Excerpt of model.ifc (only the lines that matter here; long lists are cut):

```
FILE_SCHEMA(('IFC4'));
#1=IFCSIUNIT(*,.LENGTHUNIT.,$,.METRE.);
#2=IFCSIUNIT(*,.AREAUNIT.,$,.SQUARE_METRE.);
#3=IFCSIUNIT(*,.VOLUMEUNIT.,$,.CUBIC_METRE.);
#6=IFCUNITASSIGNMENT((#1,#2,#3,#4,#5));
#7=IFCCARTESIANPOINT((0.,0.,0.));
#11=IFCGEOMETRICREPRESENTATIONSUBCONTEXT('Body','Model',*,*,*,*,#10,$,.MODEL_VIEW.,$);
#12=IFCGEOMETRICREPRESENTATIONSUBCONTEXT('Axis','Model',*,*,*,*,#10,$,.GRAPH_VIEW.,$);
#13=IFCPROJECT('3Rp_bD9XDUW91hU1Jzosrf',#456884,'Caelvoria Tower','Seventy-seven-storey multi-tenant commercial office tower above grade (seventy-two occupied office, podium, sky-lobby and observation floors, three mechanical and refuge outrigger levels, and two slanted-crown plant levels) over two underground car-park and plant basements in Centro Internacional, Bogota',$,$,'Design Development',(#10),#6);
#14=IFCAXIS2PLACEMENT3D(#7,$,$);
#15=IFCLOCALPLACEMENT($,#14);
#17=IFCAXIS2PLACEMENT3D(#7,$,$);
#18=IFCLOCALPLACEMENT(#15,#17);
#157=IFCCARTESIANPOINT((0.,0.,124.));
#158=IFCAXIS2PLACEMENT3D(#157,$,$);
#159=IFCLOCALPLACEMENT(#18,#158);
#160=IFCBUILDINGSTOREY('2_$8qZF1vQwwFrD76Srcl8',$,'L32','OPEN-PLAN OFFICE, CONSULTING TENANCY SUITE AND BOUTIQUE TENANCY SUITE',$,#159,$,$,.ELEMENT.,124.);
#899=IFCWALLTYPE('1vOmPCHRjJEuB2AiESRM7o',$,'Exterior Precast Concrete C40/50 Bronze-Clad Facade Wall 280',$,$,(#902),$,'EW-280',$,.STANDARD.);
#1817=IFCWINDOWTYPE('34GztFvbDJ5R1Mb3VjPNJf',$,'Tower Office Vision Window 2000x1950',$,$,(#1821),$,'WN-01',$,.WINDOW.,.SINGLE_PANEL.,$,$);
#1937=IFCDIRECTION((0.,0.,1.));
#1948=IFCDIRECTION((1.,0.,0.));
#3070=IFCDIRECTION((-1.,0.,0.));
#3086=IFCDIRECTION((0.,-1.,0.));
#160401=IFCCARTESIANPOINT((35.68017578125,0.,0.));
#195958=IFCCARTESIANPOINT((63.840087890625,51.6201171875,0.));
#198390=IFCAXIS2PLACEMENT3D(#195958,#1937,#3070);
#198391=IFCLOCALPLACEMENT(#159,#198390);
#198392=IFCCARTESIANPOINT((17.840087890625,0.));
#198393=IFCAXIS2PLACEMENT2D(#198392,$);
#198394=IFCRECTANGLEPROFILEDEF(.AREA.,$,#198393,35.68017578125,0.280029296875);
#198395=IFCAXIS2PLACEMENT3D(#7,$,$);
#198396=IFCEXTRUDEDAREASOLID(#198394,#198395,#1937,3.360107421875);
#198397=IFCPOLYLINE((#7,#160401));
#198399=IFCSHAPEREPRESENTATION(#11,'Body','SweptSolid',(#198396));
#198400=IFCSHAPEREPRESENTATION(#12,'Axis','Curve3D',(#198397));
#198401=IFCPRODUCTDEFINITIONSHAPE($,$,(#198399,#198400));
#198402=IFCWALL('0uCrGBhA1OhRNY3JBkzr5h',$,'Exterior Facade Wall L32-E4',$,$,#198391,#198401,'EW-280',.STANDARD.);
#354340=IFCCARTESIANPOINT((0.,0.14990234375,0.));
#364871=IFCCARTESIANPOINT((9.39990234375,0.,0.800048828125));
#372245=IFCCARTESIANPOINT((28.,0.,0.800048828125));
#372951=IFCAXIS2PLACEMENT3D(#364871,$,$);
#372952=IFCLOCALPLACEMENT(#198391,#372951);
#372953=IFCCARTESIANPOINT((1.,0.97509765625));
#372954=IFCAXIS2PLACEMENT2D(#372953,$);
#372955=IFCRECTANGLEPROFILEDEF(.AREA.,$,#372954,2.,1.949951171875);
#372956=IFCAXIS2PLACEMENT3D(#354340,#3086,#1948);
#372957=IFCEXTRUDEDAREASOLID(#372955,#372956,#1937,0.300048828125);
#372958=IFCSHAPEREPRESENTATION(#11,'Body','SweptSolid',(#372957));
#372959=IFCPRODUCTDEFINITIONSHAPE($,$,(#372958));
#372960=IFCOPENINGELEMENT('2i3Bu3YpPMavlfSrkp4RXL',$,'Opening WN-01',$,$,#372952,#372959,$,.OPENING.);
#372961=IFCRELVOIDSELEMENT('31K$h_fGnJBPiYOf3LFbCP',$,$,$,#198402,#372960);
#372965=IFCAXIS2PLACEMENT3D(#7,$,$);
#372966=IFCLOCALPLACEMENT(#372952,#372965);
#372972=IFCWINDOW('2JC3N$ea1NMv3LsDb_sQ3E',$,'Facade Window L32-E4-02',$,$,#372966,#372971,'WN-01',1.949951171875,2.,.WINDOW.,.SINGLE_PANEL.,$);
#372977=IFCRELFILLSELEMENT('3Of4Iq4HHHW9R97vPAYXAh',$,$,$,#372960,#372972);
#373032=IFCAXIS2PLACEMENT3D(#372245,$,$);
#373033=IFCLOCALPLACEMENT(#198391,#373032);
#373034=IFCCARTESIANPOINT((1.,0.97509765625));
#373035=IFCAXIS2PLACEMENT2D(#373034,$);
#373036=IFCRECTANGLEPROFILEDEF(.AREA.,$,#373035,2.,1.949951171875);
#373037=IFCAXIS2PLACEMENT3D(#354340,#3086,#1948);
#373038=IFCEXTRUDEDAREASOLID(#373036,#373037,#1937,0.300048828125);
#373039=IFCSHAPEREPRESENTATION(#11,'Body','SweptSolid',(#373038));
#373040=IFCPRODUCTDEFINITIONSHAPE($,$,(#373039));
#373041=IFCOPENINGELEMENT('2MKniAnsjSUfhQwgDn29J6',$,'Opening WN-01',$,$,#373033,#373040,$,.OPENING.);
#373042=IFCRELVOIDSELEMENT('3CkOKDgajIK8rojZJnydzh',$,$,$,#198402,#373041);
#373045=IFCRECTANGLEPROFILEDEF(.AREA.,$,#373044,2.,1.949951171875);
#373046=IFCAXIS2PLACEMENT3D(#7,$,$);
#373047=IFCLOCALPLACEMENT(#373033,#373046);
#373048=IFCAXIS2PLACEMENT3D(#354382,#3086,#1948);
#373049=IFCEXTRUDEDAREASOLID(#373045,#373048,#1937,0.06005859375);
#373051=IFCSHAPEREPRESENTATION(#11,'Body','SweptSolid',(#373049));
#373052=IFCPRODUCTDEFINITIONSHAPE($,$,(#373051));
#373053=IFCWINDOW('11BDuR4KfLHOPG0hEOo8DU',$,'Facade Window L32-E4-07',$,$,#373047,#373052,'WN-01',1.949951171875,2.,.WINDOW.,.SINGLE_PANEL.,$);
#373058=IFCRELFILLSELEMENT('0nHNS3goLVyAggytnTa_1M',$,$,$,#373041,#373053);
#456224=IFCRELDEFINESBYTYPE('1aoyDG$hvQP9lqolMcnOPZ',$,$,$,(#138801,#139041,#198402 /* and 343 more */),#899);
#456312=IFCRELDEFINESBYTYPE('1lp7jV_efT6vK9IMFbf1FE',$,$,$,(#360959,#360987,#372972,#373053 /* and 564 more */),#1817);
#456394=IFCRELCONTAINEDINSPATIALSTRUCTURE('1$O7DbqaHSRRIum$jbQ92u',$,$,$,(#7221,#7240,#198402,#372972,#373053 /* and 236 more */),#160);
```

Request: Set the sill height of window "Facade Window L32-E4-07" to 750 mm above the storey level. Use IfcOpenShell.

```python
import numpy as np
import ifcopenshell
import ifcopenshell.api.geometry
import ifcopenshell.geom
import ifcopenshell.util.element
import ifcopenshell.util.placement
import ifcopenshell.util.shape
import ifcopenshell.util.unit

model = ifcopenshell.open("model.ifc")
unit_scale = ifcopenshell.util.unit.calculate_unit_scale(model)

window = model.by_guid("11BDuR4KfLHOPG0hEOo8DU")
opening = window.FillsVoids[0].RelatingOpeningElement
storey = ifcopenshell.util.element.get_container(window, ifc_class="IfcBuildingStorey")
level = ifcopenshell.util.placement.get_local_placement(storey.ObjectPlacement)[2, 3]

# The opening's origin need not be at the sill, so measure its lowest point.
shape = ifcopenshell.geom.create_shape(ifcopenshell.geom.settings(), opening)
bottom = ifcopenshell.util.shape.get_shape_bottom_elevation(shape, shape.geometry) / unit_scale
dz = level + 0.75 - bottom

shift = np.array([0.0, 0.0, dz])
# The window is placed relative to its opening, so it follows when the opening moves.
matrix = ifcopenshell.util.placement.get_local_placement(opening.ObjectPlacement)
matrix[:3, 3] += shift
ifcopenshell.api.geometry.edit_object_placement(
    model, product=opening, matrix=matrix, is_si=False, should_transform_children=True
)

print(f"moved by {dz * unit_scale:+.3f} m")

model.write("model_v2.ifc")
```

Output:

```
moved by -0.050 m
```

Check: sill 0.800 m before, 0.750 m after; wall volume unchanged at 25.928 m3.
